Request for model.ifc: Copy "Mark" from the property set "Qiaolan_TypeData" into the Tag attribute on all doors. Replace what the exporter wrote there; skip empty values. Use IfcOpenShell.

First a look at what the model holds.

```python
import ifcopenshell
import ifcopenshell.util.element

model = ifcopenshell.open("model.ifc")
print(model.schema)
doors = model.by_type("IfcDoor")
print(len(doors), "doors")
for e in doors[:8]:
    source = ifcopenshell.util.element.get_pset(e, "Qiaolan_TypeData", "Mark")
    target = e.Tag
    print(e.id(), repr(source), repr(target), sep=" | ")
```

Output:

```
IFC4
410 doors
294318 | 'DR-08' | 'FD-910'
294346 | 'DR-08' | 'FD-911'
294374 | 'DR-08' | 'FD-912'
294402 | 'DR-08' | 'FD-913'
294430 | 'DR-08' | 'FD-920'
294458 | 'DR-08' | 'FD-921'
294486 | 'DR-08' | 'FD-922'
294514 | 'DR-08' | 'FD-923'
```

```python
import ifcopenshell
import ifcopenshell.util.element

model = ifcopenshell.open("model.ifc")

count = 0
for e in model.by_type("IfcDoor"):
    value = ifcopenshell.util.element.get_pset(e, "Qiaolan_TypeData", "Mark")
    current = e.Tag
    if not value or not value.strip() or current == value:
        continue
    e.Tag = value
    count += 1

print(count, "doors updated")

model.write("model_rev.ifc")
```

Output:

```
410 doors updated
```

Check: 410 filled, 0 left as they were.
